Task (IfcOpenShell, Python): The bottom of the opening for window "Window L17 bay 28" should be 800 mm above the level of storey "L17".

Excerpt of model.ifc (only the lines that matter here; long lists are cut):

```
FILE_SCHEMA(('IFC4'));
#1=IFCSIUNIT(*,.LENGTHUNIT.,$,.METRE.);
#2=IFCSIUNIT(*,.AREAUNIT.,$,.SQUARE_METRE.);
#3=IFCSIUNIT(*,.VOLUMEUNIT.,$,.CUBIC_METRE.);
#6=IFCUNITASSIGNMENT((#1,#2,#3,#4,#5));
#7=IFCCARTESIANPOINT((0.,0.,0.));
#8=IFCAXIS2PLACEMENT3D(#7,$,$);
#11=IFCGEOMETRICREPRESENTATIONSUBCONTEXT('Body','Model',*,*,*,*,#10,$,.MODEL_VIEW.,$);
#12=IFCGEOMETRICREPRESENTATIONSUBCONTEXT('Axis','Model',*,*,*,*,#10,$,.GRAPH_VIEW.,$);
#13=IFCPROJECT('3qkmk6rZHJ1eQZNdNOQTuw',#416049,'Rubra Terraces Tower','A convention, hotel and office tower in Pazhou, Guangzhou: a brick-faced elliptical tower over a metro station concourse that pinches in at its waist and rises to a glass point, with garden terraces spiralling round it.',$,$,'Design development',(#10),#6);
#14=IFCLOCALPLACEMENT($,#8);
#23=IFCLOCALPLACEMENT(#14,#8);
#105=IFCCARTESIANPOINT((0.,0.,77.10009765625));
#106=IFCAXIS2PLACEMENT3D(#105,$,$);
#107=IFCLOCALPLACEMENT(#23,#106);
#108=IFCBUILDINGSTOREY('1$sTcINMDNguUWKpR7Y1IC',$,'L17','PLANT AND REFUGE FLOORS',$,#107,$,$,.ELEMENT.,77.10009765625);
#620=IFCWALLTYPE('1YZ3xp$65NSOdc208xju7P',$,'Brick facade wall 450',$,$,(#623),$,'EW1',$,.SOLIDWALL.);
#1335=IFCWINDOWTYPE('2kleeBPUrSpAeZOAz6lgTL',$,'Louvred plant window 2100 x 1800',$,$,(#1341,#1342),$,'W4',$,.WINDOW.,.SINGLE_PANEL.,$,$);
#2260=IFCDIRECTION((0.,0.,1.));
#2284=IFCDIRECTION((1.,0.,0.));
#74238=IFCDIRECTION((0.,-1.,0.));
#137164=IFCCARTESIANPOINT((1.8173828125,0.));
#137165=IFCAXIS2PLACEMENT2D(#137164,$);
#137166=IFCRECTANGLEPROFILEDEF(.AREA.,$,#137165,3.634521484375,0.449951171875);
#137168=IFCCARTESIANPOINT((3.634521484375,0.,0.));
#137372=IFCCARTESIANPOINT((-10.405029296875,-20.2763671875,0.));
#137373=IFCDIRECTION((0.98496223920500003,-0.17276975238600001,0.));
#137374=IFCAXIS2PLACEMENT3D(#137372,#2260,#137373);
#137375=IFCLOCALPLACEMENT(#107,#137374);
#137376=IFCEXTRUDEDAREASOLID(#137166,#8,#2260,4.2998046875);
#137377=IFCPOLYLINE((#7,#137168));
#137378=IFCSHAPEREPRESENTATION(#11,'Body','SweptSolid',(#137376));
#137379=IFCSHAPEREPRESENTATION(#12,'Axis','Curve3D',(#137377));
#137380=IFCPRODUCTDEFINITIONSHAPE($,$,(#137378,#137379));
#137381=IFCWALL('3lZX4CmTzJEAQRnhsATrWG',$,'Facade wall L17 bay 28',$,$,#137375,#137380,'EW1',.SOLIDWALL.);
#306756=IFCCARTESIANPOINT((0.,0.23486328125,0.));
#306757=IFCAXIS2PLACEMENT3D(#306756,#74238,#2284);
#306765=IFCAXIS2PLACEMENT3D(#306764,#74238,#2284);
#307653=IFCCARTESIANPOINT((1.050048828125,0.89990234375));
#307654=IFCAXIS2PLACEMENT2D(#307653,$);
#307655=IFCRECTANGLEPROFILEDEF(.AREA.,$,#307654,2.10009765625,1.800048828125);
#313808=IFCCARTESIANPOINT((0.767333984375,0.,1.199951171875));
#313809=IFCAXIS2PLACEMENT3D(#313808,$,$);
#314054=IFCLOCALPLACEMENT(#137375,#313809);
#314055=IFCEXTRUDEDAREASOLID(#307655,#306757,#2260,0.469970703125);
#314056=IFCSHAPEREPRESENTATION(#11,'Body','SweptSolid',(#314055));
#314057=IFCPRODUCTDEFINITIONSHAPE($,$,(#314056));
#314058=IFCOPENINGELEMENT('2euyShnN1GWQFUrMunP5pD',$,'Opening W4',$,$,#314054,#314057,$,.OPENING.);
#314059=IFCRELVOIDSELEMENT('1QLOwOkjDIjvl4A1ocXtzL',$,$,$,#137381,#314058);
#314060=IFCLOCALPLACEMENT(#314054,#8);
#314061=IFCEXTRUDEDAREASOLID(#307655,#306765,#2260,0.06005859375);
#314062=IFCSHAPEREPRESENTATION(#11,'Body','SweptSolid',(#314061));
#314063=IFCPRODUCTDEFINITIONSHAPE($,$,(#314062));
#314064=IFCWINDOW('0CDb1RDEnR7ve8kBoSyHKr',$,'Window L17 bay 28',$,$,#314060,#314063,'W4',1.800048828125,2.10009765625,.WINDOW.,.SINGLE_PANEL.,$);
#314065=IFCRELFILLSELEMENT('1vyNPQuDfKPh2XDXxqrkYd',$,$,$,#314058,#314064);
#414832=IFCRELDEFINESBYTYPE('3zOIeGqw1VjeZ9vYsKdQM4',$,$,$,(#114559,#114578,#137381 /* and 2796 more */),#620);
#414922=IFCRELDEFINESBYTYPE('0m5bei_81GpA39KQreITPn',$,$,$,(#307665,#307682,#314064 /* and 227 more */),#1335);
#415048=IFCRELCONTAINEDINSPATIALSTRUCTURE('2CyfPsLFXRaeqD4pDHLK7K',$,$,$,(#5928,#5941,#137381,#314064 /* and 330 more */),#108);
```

```python
import numpy as np
import ifcopenshell
import ifcopenshell.api.geometry
import ifcopenshell.geom
import ifcopenshell.util.element
import ifcopenshell.util.placement
import ifcopenshell.util.shape
import ifcopenshell.util.unit

model = ifcopenshell.open("model.ifc")
unit_scale = ifcopenshell.util.unit.calculate_unit_scale(model)

window = model.by_guid("0CDb1RDEnR7ve8kBoSyHKr")
opening = window.FillsVoids[0].RelatingOpeningElement
storey = ifcopenshell.util.element.get_container(window, ifc_class="IfcBuildingStorey")
level = ifcopenshell.util.placement.get_local_placement(storey.ObjectPlacement)[2, 3]

# The opening's origin need not be at the sill, so measure its lowest point.
shape = ifcopenshell.geom.create_shape(ifcopenshell.geom.settings(), opening)
bottom = ifcopenshell.util.shape.get_shape_bottom_elevation(shape, shape.geometry) / unit_scale
dz = level + 0.8 - bottom

shift = np.array([0.0, 0.0, dz])
# The window is placed relative to its opening, so it follows when the opening moves.
matrix = ifcopenshell.util.placement.get_local_placement(opening.ObjectPlacement)
matrix[:3, 3] += shift
ifcopenshell.api.geometry.edit_object_placement(
    model, product=opening, matrix=matrix, is_si=False, should_transform_children=True
)

print(f"moved by {dz * unit_scale:+.3f} m")

model.write("model_v2.ifc")
```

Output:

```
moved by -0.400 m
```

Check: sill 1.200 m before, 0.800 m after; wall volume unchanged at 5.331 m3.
